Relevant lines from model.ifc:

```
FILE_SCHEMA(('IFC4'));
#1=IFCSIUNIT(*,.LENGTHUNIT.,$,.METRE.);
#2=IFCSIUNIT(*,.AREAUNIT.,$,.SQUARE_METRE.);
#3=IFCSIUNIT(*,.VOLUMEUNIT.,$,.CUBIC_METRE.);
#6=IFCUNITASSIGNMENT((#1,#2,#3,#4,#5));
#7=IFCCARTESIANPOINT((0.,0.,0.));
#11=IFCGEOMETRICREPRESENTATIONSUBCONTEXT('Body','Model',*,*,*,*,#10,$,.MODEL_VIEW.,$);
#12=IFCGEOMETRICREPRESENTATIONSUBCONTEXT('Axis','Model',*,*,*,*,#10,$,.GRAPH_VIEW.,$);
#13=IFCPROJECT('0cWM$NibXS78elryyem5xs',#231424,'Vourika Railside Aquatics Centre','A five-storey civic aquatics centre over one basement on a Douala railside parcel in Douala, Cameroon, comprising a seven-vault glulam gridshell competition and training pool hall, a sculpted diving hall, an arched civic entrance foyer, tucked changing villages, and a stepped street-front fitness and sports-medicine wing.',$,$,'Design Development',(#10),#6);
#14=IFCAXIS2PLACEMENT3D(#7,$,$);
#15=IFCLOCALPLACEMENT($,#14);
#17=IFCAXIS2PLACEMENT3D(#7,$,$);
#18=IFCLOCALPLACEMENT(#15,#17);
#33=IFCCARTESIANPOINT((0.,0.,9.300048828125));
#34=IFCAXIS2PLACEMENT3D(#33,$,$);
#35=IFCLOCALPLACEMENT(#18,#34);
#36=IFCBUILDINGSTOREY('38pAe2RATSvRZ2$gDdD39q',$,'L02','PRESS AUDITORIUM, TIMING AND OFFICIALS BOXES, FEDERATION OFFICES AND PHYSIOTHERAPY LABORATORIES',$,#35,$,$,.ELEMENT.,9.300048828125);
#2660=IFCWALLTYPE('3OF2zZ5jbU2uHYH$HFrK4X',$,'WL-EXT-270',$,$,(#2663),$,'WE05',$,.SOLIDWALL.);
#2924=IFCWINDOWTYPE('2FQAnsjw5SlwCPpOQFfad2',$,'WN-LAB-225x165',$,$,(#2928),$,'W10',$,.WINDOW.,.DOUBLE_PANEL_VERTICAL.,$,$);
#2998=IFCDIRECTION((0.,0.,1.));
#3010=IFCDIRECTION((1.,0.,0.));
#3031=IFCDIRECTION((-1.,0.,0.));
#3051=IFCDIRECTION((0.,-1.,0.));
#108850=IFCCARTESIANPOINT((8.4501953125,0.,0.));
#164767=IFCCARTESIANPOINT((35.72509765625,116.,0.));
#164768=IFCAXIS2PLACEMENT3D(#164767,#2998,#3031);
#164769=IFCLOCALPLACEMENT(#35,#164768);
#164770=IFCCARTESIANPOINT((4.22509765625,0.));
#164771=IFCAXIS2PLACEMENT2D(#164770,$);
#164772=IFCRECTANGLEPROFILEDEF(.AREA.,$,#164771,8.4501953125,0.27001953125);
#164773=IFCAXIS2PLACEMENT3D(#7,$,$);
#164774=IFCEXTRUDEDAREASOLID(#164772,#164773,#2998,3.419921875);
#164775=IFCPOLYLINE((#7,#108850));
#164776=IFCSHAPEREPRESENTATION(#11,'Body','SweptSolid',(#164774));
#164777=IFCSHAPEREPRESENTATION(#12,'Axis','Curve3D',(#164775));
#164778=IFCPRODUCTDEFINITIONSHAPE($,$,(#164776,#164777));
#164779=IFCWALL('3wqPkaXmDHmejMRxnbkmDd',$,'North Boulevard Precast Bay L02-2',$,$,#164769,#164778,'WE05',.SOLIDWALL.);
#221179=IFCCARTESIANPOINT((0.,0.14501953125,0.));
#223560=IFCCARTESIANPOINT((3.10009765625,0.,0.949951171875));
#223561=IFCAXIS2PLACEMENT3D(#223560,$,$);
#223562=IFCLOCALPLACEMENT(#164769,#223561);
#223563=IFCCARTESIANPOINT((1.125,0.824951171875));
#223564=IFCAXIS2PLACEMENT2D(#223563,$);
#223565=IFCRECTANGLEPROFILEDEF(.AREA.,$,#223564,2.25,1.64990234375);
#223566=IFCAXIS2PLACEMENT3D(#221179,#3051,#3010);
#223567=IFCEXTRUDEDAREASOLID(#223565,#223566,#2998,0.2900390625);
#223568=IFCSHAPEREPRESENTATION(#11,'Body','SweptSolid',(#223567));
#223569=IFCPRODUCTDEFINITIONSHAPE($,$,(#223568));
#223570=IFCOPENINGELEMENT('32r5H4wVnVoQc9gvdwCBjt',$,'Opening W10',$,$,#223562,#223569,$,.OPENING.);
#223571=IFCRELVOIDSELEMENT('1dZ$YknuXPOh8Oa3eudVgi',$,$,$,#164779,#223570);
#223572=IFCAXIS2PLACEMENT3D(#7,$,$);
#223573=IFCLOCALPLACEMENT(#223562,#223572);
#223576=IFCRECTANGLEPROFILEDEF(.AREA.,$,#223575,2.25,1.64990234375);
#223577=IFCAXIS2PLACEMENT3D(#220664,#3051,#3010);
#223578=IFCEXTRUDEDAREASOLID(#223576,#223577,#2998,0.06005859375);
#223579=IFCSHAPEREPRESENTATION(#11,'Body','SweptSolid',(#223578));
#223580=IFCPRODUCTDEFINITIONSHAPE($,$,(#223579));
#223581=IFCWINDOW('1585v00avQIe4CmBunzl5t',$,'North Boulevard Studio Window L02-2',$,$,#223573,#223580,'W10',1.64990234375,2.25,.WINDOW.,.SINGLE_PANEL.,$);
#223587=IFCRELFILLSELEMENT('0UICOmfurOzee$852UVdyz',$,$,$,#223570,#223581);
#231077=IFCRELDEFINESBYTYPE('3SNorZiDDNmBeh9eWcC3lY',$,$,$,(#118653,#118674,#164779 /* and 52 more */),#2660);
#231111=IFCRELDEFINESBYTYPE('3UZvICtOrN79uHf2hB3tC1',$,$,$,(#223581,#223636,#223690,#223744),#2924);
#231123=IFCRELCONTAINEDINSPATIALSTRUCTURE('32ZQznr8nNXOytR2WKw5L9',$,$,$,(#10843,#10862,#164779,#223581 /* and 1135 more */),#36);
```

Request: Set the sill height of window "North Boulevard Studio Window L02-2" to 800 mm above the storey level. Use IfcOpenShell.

```python
import numpy as np
import ifcopenshell
import ifcopenshell.api.geometry
import ifcopenshell.geom
import ifcopenshell.util.element
import ifcopenshell.util.placement
import ifcopenshell.util.shape
import ifcopenshell.util.unit

model = ifcopenshell.open("model.ifc")
unit_scale = ifcopenshell.util.unit.calculate_unit_scale(model)

window = model.by_guid("1585v00avQIe4CmBunzl5t")
opening = window.FillsVoids[0].RelatingOpeningElement
storey = ifcopenshell.util.element.get_container(window, ifc_class="IfcBuildingStorey")
level = ifcopenshell.util.placement.get_local_placement(storey.ObjectPlacement)[2, 3]

# The opening's origin need not be at the sill, so measure its lowest point.
shape = ifcopenshell.geom.create_shape(ifcopenshell.geom.settings(), opening)
bottom = ifcopenshell.util.shape.get_shape_bottom_elevation(shape, shape.geometry) / unit_scale
dz = level + 0.8 - bottom

shift = np.array([0.0, 0.0, dz])
# The window is placed relative to its opening, so it follows when the opening moves.
matrix = ifcopenshell.util.placement.get_local_placement(opening.ObjectPlacement)
matrix[:3, 3] += shift
ifcopenshell.api.geometry.edit_object_placement(
    model, product=opening, matrix=matrix, is_si=False, should_transform_children=True
)

print(f"moved by {dz * unit_scale:+.3f} m")

model.write("model_v2.ifc")
```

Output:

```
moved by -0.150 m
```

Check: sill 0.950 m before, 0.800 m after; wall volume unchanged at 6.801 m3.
